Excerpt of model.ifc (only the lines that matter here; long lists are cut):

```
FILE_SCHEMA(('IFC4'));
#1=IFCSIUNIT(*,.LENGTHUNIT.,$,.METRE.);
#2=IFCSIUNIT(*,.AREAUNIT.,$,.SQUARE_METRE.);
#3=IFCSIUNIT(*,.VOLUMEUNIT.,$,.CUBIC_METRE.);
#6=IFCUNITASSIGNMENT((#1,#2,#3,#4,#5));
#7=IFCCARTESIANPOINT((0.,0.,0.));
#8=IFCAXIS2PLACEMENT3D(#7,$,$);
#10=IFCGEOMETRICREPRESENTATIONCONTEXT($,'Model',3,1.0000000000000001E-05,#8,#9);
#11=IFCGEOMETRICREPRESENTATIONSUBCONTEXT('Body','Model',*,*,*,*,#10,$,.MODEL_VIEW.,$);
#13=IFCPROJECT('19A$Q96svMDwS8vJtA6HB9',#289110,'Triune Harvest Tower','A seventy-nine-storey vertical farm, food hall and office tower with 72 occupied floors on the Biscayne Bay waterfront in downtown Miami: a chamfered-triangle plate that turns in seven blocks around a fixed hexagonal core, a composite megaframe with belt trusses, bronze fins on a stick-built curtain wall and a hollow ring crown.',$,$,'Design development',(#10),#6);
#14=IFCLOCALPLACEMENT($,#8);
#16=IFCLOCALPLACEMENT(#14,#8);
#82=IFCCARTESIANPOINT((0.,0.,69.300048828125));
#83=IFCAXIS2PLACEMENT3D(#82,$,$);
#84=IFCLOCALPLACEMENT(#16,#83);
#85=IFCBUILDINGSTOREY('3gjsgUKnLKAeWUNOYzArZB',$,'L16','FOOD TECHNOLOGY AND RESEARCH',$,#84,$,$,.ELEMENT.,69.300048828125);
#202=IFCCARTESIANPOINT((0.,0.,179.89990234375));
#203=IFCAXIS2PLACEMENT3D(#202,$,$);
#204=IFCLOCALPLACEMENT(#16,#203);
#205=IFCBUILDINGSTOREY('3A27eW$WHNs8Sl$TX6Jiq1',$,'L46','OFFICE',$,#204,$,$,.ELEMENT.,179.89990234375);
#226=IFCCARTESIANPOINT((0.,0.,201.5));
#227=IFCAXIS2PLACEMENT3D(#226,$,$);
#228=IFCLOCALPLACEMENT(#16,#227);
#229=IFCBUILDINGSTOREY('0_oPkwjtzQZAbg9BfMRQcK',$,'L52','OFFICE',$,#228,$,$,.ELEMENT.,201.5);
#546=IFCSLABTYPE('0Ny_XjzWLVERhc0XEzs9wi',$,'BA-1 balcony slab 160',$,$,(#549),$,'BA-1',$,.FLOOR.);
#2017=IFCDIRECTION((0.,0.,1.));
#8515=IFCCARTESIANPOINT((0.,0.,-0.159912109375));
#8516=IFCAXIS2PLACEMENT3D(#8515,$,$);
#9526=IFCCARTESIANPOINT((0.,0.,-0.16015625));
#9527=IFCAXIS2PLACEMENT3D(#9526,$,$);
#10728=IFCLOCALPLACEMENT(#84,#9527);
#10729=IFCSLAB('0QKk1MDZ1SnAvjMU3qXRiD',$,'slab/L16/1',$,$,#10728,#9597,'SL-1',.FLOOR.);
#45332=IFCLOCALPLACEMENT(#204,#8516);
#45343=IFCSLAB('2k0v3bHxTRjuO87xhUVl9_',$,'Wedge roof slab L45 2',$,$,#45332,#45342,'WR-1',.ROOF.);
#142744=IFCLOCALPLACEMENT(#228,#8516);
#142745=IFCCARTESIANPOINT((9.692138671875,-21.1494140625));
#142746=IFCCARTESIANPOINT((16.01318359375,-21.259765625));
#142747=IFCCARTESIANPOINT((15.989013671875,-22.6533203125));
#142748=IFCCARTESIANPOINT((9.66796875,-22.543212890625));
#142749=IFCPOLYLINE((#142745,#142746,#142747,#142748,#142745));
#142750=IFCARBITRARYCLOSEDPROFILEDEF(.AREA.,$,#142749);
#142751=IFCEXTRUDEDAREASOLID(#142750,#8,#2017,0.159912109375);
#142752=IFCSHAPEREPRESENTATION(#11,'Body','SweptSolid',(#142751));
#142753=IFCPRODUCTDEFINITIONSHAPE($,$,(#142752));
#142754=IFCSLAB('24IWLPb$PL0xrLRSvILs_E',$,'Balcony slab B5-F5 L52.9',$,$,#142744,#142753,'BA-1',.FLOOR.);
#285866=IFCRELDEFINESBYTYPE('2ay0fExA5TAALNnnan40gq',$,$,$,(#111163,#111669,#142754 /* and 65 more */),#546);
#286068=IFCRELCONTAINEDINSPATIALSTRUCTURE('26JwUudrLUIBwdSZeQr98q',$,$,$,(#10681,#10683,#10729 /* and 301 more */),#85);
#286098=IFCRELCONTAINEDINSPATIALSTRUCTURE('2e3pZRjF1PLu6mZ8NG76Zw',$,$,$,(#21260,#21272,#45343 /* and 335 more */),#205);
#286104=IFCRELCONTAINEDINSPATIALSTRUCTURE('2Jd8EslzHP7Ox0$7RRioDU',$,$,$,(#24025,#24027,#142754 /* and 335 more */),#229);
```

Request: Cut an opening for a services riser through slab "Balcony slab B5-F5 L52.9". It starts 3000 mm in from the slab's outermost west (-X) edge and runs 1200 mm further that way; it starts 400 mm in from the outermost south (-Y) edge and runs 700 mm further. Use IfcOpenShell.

```python
import numpy as np
import ifcopenshell
import ifcopenshell.api.feature
import ifcopenshell.api.geometry
import ifcopenshell.api.root
import ifcopenshell.geom
import ifcopenshell.util.placement
import ifcopenshell.util.representation
import ifcopenshell.util.shape
import ifcopenshell.util.unit

model = ifcopenshell.open("model.ifc")
unit_scale = ifcopenshell.util.unit.calculate_unit_scale(model)
settings = ifcopenshell.geom.settings()


def volume(element):
    """Net volume in cubic metres, openings subtracted."""
    shape = ifcopenshell.geom.create_shape(settings, element)
    return ifcopenshell.util.shape.get_volume(shape.geometry)


slab = model.by_guid("24IWLPb$PL0xrLRSvILs_E")
before = volume(slab)

# Extent in the slab's own axes, in metres. The edges named are its -X and -Y sides.
slab_shape = ifcopenshell.geom.create_shape(settings, slab)
vertices = ifcopenshell.util.shape.get_vertices(slab_shape.geometry)
x_min, y_min, bottom = vertices.min(axis=0)
top = vertices[:, 2].max()

opening = ifcopenshell.api.root.create_entity(model, ifc_class="IfcOpeningElement", name="Services riser opening", predefined_type="OPENING")
context = ifcopenshell.util.representation.get_context(model, "Model", "Body", "MODEL_VIEW")
width, depth = 1.2, 0.7
outline = [(0.0, 0.0), (width, 0.0), (width, depth), (0.0, depth), (0.0, 0.0)]
# Overshoot both faces by 50 mm so the cut is clean.
shape = ifcopenshell.api.geometry.add_slab_representation(
    model, context=context, depth=top - bottom + 0.1, polyline=outline
)
ifcopenshell.api.geometry.assign_representation(model, product=opening, representation=shape)

matrix = ifcopenshell.util.placement.get_local_placement(slab.ObjectPlacement)
matrix[:, 3] = matrix @ np.append(np.array([x_min + 3, y_min + 0.4, bottom - 0.05]) / unit_scale, 1.0)
ifcopenshell.api.geometry.edit_object_placement(model, product=opening, matrix=matrix, is_si=False)
ifcopenshell.api.feature.add_feature(model, feature=opening, element=slab)

after = volume(slab)

print(f"slab volume {before:.3f} -> {after:.3f} m3")

model.write("model_updated.ifc")
```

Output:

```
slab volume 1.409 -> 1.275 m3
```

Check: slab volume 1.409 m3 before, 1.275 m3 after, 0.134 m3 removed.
